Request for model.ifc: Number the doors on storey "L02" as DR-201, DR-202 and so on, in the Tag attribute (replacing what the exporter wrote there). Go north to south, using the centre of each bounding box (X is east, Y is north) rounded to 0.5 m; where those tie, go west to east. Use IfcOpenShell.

First a look at what the model holds.

```python
import ifcopenshell
import ifcopenshell.util.element
import ifcopenshell.util.placement

model = ifcopenshell.open("model.ifc")
print(model.schema)
storey = next(s for s in model.by_type("IfcBuildingStorey") if s.Name == "L02")
doors = [e for e in ifcopenshell.util.element.get_decomposition(storey) if e.is_a("IfcDoor")]
for e in sorted(doors, key=lambda e: e.id()):
    origin = ifcopenshell.util.placement.get_local_placement(e.ObjectPlacement)[:3, 3]
    print(e.id(), e.Tag, e.Name, origin.round(2) + 0.0, sep=" | ")
```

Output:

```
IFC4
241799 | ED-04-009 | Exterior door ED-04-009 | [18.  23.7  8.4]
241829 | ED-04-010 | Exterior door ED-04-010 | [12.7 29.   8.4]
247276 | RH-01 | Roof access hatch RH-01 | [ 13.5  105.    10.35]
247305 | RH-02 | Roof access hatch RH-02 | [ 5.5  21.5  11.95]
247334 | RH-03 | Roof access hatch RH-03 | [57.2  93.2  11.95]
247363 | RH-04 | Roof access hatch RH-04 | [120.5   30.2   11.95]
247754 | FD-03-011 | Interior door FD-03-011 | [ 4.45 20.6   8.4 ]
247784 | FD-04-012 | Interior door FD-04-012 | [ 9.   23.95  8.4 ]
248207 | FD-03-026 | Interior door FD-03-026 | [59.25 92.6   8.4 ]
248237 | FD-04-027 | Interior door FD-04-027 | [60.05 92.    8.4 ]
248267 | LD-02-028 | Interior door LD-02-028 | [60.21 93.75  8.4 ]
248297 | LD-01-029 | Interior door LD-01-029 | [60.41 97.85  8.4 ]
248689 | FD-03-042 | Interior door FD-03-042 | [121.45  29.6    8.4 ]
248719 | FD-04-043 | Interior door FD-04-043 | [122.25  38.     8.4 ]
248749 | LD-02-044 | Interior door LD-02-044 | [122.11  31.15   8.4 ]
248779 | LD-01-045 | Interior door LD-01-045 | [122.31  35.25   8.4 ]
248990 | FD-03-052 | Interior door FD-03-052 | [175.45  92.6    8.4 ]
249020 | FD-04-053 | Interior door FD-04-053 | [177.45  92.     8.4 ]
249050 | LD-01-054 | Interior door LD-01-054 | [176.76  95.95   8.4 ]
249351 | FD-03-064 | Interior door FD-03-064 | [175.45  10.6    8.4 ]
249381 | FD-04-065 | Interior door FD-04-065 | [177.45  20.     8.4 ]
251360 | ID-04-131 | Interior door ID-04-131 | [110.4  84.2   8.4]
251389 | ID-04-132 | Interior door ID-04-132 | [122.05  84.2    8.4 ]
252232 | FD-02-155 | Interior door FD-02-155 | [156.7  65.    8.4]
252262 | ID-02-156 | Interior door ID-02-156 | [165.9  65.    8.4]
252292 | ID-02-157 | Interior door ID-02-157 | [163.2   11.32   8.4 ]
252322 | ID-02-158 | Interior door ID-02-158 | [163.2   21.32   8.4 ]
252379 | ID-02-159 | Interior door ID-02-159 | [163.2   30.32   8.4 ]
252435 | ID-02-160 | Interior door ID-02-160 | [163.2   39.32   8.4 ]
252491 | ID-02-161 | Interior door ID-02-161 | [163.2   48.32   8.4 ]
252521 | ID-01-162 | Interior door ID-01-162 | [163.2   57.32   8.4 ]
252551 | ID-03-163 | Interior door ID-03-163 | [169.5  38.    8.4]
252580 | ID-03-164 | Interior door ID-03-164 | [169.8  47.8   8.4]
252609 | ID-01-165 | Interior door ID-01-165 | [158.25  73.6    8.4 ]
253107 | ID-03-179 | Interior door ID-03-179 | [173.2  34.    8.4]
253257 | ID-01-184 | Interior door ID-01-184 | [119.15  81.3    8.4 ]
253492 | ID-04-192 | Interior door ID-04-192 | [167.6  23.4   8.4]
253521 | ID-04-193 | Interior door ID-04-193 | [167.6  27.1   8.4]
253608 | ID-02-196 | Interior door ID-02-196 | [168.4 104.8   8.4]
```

```python
import ifcopenshell
import ifcopenshell.geom
import ifcopenshell.util.element
import ifcopenshell.util.shape

model = ifcopenshell.open("model.ifc")
settings = ifcopenshell.geom.settings()
settings.set("use-world-coords", True)


def centre(element):
    shape = ifcopenshell.geom.create_shape(settings, element)
    return ifcopenshell.util.shape.get_bbox_centroid(shape.geometry)


storey = next(s for s in model.by_type("IfcBuildingStorey") if s.Name == "L02")
doors = [e for e in ifcopenshell.util.element.get_decomposition(storey) if e.is_a("IfcDoor")]

# Insertion points can sit at a corner or the storey origin, so sort by the geometry (in metres).
centres = {e: centre(e) for e in doors}
doors.sort(key=lambda e: (-round(centres[e][1] / 0.5), centres[e][0]))

for i, e in enumerate(doors, start=1):
    number = f"DR-2{i:02d}"
    e.Tag = number
    print(e.id(), number)

model.write("model_v2.ifc")
```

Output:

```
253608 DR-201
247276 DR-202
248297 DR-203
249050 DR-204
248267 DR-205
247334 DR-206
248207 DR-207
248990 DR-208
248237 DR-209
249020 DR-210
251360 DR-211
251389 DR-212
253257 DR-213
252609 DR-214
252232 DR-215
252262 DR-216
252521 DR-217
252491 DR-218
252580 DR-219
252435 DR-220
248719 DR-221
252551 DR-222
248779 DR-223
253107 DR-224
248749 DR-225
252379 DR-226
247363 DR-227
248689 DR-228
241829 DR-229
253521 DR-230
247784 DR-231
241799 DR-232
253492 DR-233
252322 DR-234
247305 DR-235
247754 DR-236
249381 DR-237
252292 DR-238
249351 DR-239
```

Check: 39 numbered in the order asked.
